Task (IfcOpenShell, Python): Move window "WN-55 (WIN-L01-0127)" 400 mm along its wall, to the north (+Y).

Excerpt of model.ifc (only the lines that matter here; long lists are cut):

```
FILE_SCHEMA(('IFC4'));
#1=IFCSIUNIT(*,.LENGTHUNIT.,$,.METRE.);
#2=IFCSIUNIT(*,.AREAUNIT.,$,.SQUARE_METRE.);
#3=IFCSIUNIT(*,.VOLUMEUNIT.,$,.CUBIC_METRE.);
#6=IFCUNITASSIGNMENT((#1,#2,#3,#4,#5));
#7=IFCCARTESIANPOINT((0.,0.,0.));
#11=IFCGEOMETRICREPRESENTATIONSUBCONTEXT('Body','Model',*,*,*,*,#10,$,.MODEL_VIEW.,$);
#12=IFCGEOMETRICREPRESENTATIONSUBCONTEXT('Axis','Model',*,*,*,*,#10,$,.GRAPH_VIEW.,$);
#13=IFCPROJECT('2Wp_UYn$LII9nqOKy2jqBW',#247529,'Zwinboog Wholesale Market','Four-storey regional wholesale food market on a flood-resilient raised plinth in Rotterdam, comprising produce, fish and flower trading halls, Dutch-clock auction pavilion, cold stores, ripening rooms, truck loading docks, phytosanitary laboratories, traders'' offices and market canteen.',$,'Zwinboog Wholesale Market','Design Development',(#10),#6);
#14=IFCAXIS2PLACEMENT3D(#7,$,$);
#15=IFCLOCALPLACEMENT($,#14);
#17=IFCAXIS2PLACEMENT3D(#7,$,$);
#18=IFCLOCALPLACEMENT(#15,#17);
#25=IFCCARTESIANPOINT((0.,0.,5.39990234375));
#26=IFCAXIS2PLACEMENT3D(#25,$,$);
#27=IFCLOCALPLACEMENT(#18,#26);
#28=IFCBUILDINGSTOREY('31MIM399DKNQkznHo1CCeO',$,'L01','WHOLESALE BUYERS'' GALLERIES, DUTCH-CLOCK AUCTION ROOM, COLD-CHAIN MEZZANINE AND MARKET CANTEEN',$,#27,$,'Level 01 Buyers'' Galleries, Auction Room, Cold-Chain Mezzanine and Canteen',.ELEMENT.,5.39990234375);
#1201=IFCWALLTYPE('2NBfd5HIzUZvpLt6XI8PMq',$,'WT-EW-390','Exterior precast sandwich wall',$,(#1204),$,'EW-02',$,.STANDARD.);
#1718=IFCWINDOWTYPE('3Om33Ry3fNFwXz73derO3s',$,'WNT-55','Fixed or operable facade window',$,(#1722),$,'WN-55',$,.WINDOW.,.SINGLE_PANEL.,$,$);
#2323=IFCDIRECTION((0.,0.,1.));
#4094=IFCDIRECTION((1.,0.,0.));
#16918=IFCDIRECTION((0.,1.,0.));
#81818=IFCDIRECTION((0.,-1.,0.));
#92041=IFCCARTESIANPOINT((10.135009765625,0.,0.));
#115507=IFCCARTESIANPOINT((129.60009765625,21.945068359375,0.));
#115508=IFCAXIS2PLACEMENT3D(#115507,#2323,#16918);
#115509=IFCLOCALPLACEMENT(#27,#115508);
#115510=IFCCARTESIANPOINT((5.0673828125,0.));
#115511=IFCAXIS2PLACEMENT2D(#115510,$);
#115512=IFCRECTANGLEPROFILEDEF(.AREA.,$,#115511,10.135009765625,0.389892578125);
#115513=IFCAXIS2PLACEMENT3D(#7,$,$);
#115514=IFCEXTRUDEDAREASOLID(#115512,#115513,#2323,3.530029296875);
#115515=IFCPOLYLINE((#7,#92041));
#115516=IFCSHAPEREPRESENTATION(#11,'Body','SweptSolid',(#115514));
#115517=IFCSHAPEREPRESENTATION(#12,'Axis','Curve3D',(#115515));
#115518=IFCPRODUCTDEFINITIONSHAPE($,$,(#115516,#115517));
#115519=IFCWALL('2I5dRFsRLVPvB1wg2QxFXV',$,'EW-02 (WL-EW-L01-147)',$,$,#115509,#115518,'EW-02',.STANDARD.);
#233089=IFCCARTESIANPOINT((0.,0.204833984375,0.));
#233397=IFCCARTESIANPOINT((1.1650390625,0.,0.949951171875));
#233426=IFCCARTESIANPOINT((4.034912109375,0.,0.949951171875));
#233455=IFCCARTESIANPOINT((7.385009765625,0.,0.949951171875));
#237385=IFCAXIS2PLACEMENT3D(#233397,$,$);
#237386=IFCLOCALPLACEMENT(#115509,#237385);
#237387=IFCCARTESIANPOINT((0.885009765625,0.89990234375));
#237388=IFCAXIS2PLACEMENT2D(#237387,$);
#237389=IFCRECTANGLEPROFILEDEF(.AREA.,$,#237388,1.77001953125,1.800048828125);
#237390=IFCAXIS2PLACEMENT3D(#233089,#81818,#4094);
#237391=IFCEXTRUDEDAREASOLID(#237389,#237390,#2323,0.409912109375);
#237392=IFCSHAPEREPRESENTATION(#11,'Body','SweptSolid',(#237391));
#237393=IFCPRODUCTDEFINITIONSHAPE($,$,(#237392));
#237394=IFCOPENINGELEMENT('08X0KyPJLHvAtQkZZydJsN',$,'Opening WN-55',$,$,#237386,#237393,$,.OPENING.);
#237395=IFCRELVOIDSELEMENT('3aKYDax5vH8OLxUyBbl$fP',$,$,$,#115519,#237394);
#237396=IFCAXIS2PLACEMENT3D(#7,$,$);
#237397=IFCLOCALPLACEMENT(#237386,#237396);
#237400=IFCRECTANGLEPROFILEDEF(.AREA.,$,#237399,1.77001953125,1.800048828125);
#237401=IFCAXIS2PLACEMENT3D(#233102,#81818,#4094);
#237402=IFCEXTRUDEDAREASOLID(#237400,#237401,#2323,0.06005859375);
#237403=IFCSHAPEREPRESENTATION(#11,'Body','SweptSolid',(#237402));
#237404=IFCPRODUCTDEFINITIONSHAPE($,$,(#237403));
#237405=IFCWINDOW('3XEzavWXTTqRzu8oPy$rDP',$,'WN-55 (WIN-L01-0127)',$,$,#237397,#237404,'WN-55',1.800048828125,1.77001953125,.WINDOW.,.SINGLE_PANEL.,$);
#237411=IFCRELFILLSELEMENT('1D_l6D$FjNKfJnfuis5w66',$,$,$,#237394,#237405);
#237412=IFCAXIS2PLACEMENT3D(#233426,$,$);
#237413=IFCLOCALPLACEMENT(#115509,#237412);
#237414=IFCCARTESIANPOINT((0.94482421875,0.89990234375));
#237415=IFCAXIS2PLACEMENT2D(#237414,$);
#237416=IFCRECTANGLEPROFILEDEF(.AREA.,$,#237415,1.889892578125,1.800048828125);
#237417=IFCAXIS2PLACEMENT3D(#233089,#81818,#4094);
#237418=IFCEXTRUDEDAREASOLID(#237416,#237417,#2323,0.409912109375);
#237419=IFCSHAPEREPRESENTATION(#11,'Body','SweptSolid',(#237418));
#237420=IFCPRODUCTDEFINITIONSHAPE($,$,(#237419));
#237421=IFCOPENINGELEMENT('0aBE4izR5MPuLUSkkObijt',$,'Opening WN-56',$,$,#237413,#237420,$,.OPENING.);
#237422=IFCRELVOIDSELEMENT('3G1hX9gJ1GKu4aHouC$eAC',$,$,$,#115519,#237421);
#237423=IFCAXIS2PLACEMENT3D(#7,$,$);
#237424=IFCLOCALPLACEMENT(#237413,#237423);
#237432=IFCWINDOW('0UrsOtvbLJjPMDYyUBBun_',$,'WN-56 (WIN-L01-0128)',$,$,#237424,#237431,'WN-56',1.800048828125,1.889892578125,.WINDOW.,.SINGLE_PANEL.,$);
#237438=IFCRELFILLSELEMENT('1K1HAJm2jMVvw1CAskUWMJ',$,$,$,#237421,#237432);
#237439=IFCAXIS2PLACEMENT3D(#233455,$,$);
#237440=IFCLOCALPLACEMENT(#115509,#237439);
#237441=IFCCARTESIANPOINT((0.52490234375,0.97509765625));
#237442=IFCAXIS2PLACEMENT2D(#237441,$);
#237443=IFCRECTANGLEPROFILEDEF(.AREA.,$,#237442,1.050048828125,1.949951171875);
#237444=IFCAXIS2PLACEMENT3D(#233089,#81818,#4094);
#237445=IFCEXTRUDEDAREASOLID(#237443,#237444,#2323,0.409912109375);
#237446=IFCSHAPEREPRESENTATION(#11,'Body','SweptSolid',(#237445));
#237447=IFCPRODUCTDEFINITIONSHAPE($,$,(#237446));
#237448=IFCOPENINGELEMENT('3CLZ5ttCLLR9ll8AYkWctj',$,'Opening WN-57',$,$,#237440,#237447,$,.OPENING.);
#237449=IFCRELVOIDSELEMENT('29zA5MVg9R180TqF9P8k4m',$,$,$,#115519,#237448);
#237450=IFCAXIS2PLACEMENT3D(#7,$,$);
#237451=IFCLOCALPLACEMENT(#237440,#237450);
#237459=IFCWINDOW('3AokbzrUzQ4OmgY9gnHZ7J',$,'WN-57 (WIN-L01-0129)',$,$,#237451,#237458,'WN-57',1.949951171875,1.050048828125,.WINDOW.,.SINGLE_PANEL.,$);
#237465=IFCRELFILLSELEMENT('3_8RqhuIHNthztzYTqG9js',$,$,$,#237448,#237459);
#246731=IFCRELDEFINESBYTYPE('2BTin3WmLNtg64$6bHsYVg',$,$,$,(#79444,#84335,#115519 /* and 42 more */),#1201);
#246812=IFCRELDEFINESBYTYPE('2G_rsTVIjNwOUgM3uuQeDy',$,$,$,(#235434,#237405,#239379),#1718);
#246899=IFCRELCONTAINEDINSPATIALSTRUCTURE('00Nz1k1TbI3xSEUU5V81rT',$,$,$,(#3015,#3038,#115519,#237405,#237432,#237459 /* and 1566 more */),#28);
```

```python
import ifcopenshell
import ifcopenshell.api.geometry
import ifcopenshell.util.placement

model = ifcopenshell.open("model.ifc")

window = model.by_guid("3XEzavWXTTqRzu8oPy$rDP")
opening = window.FillsVoids[0].RelatingOpeningElement
wall = opening.VoidsElements[0].RelatingBuildingElement

wall_matrix = ifcopenshell.util.placement.get_local_placement(wall.ObjectPlacement)
shift = wall_matrix[:3, 0] * 0.4
before = ifcopenshell.util.placement.get_local_placement(window.ObjectPlacement)[:3, 3].copy()

# The window is placed relative to its opening, so it follows when the opening moves.
matrix = ifcopenshell.util.placement.get_local_placement(opening.ObjectPlacement)
matrix[:3, 3] += shift
ifcopenshell.api.geometry.edit_object_placement(
    model, product=opening, matrix=matrix, is_si=False, should_transform_children=True
)

after = ifcopenshell.util.placement.get_local_placement(window.ObjectPlacement)[:3, 3]
print("window moved by", (after - before).round(3) + 0.0)

model.write("model_edited.ifc")
```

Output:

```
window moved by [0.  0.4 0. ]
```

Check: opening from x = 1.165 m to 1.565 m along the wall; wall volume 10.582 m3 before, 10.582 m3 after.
